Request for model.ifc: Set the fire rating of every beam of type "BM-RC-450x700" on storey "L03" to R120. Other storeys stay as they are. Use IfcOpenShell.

First a look at what the model holds.

```python
import ifcopenshell
import ifcopenshell.util.element

model = ifcopenshell.open("model.ifc")
print(model.schema)
storey = next(s for s in model.by_type("IfcBuildingStorey") if s.Name == "L03")
beams = [e for e in ifcopenshell.util.element.get_decomposition(storey) if e.is_a("IfcBeam")]
seen = {}
for e in beams:
    element_type = ifcopenshell.util.element.get_type(e)
    key = (element_type.Name if element_type != e and element_type else None, ifcopenshell.util.element.get_pset(e, "Pset_BeamCommon", "FireRating"))
    seen[key] = seen.get(key, 0) + 1
for (name, value), count in sorted(seen.items(), key=str):
    print(count, "x", name, "|", value)
```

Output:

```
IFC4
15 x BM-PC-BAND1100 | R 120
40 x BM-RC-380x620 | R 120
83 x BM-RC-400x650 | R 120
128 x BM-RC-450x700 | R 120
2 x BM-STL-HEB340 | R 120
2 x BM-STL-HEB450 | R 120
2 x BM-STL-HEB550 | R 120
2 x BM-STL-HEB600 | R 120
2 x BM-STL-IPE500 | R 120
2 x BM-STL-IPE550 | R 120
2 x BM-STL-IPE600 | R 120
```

```python
import ifcopenshell
import ifcopenshell.api.pset
import ifcopenshell.util.element

model = ifcopenshell.open("model.ifc")

storey = next(s for s in model.by_type("IfcBuildingStorey") if s.Name == "L03")
beams = [e for e in ifcopenshell.util.element.get_decomposition(storey) if e.is_a("IfcBeam")]

count = 0
for e in beams:
    element_type = ifcopenshell.util.element.get_type(e)
    if element_type in (None, e) or element_type.Name != "BM-RC-450x700":
        continue
    # add_pset returns the element's existing set when there is one.
    pset = ifcopenshell.api.pset.add_pset(model, product=e, name="Pset_BeamCommon")
    ifcopenshell.api.pset.edit_pset(model, pset=pset, properties={"FireRating": "R120"})
    count += 1

print(count, "beams updated")

model.write("model_edited.ifc")
```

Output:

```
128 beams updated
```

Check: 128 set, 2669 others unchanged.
